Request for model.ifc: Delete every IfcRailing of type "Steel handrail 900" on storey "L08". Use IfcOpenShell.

First a look at what the model holds.

```python
import ifcopenshell
import ifcopenshell.util.element

model = ifcopenshell.open("model.ifc")
print(model.schema)
storey = next(s for s in model.by_type("IfcBuildingStorey") if s.Name == "L08")
railings = [e for e in ifcopenshell.util.element.get_decomposition(storey) if e.is_a("IfcRailing")]
seen = {}
for e in railings:
    element_type = ifcopenshell.util.element.get_type(e)
    name = element_type.Name if element_type not in (None, e) else None
    seen[name] = seen.get(name, 0) + 1
for name, count in sorted(seen.items(), key=str):
    print(count, "x", name)
```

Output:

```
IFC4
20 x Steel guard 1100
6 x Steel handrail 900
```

```python
import ifcopenshell
import ifcopenshell.api.root
import ifcopenshell.util.element

model = ifcopenshell.open("model.ifc")

storey = next(s for s in model.by_type("IfcBuildingStorey") if s.Name == "L08")
railings = [e for e in ifcopenshell.util.element.get_decomposition(storey) if e.is_a("IfcRailing")]
targets = [e for e in railings if (t := ifcopenshell.util.element.get_type(e)) not in (None, e) and t.Name == "Steel handrail 900"]

for e in targets:
    ifcopenshell.api.root.remove_product(model, product=e)
print(len(targets), "removed")

model.write("model_rev.ifc")
```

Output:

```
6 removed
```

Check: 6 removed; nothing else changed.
